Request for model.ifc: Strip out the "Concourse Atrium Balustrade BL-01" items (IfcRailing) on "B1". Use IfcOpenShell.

First a look at what the model holds.

```python
import ifcopenshell
import ifcopenshell.util.element

model = ifcopenshell.open("model.ifc")
print(model.schema)
storey = next(s for s in model.by_type("IfcBuildingStorey") if s.Name == "B1")
railings = [e for e in ifcopenshell.util.element.get_decomposition(storey) if e.is_a("IfcRailing")]
seen = {}
for e in railings:
    element_type = ifcopenshell.util.element.get_type(e)
    name = element_type.Name if element_type not in (None, e) else None
    seen[name] = seen.get(name, 0) + 1
for name, count in sorted(seen.items(), key=str):
    print(count, "x", name)
```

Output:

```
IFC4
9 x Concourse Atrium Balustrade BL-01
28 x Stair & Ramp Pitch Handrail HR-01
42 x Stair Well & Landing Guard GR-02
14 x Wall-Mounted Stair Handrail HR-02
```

```python
import ifcopenshell
import ifcopenshell.api.root
import ifcopenshell.util.element

model = ifcopenshell.open("model.ifc")

storey = next(s for s in model.by_type("IfcBuildingStorey") if s.Name == "B1")
railings = [e for e in ifcopenshell.util.element.get_decomposition(storey) if e.is_a("IfcRailing")]
targets = [e for e in railings if (t := ifcopenshell.util.element.get_type(e)) not in (None, e) and t.Name == "Concourse Atrium Balustrade BL-01"]

for e in targets:
    ifcopenshell.api.root.remove_product(model, product=e)
print(len(targets), "removed")

model.write("model_v2.ifc")
```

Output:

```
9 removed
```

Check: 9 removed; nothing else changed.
